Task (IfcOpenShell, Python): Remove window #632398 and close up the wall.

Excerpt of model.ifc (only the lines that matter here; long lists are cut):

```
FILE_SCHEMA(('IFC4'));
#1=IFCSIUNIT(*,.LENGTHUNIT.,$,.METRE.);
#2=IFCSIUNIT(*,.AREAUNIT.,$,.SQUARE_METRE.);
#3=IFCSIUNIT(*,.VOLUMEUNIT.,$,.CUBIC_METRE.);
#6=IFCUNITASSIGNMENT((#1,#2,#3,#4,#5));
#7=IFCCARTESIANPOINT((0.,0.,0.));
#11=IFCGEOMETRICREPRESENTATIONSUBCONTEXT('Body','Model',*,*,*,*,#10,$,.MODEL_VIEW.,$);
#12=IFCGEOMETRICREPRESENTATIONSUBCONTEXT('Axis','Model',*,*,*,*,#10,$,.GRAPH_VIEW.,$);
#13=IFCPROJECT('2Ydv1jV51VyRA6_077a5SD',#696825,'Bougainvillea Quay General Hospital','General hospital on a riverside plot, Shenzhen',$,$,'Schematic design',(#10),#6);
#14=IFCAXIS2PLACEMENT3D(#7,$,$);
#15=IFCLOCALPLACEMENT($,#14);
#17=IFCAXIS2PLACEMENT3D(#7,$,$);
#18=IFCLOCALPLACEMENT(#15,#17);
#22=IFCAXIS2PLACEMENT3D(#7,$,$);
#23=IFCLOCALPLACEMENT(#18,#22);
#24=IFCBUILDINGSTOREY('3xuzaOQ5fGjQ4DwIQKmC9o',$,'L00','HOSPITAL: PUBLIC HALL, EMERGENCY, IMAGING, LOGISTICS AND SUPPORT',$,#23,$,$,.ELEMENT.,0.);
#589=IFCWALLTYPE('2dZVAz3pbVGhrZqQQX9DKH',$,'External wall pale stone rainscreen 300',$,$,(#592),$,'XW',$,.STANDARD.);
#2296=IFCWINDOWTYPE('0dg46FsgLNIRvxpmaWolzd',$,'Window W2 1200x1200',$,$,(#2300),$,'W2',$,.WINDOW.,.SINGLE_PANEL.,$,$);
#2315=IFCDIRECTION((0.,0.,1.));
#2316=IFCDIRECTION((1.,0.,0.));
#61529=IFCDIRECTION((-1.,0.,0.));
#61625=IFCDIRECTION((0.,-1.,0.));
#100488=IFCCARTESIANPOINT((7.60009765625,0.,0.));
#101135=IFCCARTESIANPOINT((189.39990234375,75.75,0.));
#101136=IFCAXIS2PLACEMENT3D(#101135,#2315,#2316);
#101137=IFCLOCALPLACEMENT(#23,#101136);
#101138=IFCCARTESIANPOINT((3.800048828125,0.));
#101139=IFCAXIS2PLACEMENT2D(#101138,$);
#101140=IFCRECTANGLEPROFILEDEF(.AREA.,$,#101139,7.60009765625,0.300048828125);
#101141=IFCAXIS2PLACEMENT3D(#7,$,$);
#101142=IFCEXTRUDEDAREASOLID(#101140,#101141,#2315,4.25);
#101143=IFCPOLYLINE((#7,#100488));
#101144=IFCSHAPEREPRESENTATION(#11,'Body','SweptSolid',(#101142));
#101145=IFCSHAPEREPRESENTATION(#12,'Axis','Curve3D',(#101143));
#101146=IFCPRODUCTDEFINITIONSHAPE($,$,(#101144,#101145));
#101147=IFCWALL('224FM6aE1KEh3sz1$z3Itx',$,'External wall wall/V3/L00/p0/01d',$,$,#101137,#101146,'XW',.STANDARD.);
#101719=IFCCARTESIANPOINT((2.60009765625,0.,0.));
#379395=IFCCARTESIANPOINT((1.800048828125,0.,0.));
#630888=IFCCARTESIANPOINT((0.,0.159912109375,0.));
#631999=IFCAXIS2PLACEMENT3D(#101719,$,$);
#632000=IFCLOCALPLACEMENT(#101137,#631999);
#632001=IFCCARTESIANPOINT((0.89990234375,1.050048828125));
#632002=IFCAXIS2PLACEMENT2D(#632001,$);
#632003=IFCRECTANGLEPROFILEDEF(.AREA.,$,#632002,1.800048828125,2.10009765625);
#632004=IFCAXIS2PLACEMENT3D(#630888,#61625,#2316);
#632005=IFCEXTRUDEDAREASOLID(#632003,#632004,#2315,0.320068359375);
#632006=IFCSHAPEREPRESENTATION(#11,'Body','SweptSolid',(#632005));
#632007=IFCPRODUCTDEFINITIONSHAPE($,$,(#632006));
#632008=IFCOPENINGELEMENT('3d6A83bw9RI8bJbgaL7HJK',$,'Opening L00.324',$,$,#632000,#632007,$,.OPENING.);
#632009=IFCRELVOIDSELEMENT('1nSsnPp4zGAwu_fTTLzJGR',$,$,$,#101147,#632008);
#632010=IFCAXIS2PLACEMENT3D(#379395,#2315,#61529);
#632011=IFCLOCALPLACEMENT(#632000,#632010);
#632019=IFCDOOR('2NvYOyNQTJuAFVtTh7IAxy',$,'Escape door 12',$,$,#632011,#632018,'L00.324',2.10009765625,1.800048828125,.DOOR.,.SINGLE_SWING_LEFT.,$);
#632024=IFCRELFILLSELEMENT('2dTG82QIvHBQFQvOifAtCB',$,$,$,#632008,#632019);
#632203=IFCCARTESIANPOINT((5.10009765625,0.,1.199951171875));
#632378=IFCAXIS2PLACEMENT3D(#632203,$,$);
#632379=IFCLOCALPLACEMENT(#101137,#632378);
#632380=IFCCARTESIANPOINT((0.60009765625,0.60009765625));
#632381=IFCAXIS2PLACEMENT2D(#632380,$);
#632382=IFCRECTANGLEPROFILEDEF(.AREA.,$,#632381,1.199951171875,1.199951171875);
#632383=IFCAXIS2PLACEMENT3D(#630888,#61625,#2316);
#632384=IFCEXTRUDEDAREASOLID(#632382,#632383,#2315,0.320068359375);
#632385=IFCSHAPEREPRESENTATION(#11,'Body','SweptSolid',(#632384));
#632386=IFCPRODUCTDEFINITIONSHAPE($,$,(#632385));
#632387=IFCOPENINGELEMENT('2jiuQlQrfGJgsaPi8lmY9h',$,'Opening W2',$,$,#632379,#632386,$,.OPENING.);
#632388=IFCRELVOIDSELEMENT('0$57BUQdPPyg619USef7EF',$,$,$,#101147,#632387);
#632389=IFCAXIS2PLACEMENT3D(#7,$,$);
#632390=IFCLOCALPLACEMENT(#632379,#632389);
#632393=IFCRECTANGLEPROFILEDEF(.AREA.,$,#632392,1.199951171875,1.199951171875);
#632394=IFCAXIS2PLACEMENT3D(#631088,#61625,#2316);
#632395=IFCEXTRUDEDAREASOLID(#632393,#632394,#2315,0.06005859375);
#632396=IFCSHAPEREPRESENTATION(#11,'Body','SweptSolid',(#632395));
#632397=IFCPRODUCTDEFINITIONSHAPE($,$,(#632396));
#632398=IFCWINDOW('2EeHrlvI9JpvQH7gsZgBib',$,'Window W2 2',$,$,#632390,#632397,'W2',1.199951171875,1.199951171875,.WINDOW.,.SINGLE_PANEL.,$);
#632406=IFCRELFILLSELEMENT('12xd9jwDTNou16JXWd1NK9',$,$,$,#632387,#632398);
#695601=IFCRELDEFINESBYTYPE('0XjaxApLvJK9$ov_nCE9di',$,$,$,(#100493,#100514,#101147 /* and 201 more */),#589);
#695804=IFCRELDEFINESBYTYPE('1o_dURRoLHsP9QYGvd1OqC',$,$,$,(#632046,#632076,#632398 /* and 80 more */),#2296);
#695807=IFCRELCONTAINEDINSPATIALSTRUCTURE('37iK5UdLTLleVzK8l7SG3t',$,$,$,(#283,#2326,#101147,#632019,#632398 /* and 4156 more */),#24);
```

```python
import ifcopenshell
import ifcopenshell.api.feature
import ifcopenshell.api.root
import ifcopenshell.geom
import ifcopenshell.util.shape

model = ifcopenshell.open("model.ifc")
settings = ifcopenshell.geom.settings()


def volume(element):
    """Net volume in cubic metres, openings subtracted."""
    shape = ifcopenshell.geom.create_shape(settings, element)
    return ifcopenshell.util.shape.get_volume(shape.geometry)


window = model.by_guid("2EeHrlvI9JpvQH7gsZgBib")
opening = window.FillsVoids[0].RelatingOpeningElement
wall = opening.VoidsElements[0].RelatingBuildingElement
before = volume(wall)

ifcopenshell.api.root.remove_product(model, product=window)
ifcopenshell.api.feature.remove_feature(model, feature=opening)

after = volume(wall)

print(f"wall volume {before:.3f} -> {after:.3f} m3")

model.write("model-out.ifc")
```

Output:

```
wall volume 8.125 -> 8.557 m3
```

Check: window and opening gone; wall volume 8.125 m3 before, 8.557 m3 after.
